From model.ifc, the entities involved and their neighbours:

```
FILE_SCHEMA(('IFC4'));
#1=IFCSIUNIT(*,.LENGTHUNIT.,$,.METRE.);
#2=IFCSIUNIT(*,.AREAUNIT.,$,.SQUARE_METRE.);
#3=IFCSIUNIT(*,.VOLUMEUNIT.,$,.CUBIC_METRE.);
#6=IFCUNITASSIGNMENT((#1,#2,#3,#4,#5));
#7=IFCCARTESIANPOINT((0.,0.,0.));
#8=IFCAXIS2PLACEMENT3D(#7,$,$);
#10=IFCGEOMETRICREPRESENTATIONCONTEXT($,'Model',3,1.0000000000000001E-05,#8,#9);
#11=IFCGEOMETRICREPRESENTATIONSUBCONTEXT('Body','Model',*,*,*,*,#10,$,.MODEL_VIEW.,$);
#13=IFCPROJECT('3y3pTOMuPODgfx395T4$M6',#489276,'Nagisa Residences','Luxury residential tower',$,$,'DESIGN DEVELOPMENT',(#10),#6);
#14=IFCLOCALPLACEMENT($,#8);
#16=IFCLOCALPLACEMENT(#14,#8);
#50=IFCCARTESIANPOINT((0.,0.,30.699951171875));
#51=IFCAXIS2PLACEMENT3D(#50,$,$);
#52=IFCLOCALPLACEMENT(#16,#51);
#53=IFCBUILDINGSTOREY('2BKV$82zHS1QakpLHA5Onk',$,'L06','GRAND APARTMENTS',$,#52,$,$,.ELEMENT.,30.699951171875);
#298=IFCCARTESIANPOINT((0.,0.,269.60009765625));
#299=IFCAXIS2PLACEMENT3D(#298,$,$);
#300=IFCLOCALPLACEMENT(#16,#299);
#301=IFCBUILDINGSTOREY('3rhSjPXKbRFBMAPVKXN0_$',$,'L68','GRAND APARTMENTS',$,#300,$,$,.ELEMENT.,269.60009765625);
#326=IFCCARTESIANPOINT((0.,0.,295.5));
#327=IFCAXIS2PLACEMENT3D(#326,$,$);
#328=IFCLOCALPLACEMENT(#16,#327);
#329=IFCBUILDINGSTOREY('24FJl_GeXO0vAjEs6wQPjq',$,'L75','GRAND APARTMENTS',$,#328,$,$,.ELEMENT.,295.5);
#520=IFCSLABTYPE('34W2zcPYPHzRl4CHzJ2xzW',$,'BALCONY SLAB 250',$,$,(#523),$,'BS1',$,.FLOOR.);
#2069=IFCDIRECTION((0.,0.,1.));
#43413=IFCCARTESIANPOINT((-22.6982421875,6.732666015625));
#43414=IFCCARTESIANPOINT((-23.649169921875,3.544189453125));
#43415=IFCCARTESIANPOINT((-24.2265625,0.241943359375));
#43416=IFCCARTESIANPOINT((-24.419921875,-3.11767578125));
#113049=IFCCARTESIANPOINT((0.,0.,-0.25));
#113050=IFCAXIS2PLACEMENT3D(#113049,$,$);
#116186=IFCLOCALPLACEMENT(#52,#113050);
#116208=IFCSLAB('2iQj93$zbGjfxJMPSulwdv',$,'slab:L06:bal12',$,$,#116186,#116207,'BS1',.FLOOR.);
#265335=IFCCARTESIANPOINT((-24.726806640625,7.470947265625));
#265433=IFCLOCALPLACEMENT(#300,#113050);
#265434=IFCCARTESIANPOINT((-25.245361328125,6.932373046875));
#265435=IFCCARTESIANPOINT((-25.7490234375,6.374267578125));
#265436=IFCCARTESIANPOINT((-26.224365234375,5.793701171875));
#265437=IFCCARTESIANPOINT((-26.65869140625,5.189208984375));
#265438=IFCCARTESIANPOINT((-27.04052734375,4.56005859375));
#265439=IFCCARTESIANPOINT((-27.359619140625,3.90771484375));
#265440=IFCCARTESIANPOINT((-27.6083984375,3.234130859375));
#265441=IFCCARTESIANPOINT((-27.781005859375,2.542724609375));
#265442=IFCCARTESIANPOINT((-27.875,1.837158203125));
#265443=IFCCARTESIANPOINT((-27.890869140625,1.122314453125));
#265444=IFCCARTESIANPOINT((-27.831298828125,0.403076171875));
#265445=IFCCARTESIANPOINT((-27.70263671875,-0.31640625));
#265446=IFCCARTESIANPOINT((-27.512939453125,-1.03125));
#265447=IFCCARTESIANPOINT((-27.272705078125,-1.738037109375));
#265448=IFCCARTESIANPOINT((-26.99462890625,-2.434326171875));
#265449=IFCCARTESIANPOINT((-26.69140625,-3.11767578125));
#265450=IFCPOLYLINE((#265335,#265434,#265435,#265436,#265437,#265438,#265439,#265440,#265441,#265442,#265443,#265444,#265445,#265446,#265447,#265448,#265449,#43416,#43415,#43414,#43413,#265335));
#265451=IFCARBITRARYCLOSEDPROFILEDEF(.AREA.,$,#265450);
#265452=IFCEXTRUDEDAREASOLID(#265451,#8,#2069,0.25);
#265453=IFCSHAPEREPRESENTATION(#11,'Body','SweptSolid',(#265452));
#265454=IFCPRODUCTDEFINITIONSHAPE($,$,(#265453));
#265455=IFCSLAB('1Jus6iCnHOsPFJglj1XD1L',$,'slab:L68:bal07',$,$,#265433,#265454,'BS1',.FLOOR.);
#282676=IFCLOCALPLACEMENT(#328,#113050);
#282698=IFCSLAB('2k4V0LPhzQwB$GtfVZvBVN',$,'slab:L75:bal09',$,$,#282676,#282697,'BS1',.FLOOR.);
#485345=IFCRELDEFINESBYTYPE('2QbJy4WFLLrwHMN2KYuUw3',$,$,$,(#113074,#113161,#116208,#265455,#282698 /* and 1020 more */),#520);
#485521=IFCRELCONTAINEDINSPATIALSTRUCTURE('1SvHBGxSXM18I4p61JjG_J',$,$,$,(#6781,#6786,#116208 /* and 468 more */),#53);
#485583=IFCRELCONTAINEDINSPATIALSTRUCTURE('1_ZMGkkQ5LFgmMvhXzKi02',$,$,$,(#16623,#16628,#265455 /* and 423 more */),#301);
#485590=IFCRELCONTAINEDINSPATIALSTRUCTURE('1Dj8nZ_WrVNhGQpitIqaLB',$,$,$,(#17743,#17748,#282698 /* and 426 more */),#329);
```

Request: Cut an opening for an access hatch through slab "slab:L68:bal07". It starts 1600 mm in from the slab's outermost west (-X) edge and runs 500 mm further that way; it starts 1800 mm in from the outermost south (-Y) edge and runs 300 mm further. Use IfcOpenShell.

```python
import numpy as np
import ifcopenshell
import ifcopenshell.api.feature
import ifcopenshell.api.geometry
import ifcopenshell.api.root
import ifcopenshell.geom
import ifcopenshell.util.placement
import ifcopenshell.util.representation
import ifcopenshell.util.shape
import ifcopenshell.util.unit

model = ifcopenshell.open("model.ifc")
unit_scale = ifcopenshell.util.unit.calculate_unit_scale(model)
settings = ifcopenshell.geom.settings()


def volume(element):
    """Net volume in cubic metres, openings subtracted."""
    shape = ifcopenshell.geom.create_shape(settings, element)
    return ifcopenshell.util.shape.get_volume(shape.geometry)


slab = model.by_id(265455)
before = volume(slab)

# Extent in the slab's own axes, in metres. The edges named are its -X and -Y sides.
slab_shape = ifcopenshell.geom.create_shape(settings, slab)
vertices = ifcopenshell.util.shape.get_vertices(slab_shape.geometry)
x_min, y_min, bottom = vertices.min(axis=0)
top = vertices[:, 2].max()

opening = ifcopenshell.api.root.create_entity(model, ifc_class="IfcOpeningElement", name="Access hatch opening", predefined_type="OPENING")
context = ifcopenshell.util.representation.get_context(model, "Model", "Body", "MODEL_VIEW")
width, depth = 0.5, 0.3
outline = [(0.0, 0.0), (width, 0.0), (width, depth), (0.0, depth), (0.0, 0.0)]
# Overshoot both faces by 50 mm so the cut is clean.
shape = ifcopenshell.api.geometry.add_slab_representation(
    model, context=context, depth=top - bottom + 0.1, polyline=outline
)
ifcopenshell.api.geometry.assign_representation(model, product=opening, representation=shape)

matrix = ifcopenshell.util.placement.get_local_placement(slab.ObjectPlacement)
matrix[:, 3] = matrix @ np.append(np.array([x_min + 1.6, y_min + 1.8, bottom - 0.05]) / unit_scale, 1.0)
ifcopenshell.api.geometry.edit_object_placement(model, product=opening, matrix=matrix, is_si=False)
ifcopenshell.api.feature.add_feature(model, feature=opening, element=slab)

after = volume(slab)

print(f"slab volume {before:.3f} -> {after:.3f} m3")

model.write("model_v2.ifc")
```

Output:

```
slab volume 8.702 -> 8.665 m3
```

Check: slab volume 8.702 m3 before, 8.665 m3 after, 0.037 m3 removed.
